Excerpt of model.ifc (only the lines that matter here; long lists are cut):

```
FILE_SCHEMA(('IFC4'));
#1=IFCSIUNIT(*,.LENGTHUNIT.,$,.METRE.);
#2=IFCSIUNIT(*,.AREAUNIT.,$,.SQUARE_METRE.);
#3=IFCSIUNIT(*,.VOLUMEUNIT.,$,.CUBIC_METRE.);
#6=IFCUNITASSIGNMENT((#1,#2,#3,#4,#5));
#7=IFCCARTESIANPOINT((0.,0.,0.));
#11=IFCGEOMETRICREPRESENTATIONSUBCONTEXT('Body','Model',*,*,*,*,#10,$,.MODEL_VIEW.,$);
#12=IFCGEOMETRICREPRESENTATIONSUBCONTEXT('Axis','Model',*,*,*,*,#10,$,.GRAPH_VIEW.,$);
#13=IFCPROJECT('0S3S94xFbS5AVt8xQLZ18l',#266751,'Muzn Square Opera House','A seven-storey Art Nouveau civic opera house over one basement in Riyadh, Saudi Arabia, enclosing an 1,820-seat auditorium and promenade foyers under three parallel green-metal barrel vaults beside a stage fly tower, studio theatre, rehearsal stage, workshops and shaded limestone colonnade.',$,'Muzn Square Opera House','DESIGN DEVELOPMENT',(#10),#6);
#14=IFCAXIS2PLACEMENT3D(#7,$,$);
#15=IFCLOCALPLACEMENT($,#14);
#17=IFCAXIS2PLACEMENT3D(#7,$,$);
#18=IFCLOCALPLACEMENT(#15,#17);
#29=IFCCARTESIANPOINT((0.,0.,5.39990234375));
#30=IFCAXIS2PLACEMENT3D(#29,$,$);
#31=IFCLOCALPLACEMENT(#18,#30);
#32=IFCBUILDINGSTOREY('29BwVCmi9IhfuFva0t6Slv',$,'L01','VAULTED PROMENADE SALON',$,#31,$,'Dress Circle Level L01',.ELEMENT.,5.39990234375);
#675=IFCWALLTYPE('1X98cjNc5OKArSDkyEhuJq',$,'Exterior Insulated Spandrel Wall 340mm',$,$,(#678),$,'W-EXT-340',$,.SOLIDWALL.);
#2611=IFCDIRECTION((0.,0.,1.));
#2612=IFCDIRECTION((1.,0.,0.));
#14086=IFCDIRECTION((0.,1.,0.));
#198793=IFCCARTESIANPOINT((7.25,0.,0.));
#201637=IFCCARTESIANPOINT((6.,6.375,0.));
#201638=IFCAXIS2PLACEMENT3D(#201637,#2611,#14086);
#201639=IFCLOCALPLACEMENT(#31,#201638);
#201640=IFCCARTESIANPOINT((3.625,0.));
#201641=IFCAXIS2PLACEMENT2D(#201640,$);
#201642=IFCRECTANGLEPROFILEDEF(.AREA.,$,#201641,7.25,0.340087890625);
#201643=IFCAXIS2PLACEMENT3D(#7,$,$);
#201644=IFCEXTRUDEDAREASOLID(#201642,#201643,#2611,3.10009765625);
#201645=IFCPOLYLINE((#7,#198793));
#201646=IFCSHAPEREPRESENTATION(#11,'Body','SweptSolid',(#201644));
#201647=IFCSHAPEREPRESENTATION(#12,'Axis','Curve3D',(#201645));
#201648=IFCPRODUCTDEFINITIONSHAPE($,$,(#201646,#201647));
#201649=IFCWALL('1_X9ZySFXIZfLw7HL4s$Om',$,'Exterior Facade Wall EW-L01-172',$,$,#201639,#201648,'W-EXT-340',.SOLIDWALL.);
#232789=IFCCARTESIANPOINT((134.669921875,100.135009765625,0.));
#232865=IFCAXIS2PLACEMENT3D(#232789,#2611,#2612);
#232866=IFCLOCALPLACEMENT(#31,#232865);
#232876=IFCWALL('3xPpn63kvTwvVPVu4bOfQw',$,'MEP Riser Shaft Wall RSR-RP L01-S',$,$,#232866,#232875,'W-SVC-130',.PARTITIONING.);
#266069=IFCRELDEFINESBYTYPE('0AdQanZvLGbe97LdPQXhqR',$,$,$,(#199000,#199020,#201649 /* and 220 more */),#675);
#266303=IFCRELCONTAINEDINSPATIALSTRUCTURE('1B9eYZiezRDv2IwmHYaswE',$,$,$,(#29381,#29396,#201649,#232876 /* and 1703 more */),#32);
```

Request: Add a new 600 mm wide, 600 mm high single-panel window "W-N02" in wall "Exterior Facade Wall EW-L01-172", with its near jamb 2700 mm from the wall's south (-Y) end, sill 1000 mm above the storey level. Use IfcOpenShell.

```python
import numpy as np
import ifcopenshell
import ifcopenshell.api.feature
import ifcopenshell.api.geometry
import ifcopenshell.api.root
import ifcopenshell.api.spatial
import ifcopenshell.geom
import ifcopenshell.util.element
import ifcopenshell.util.placement
import ifcopenshell.util.representation
import ifcopenshell.util.shape
import ifcopenshell.util.unit

model = ifcopenshell.open("model.ifc")
unit_scale = ifcopenshell.util.unit.calculate_unit_scale(model)
settings = ifcopenshell.geom.settings()


def volume(element):
    """Net volume in cubic metres, openings subtracted."""
    shape = ifcopenshell.geom.create_shape(settings, element)
    return ifcopenshell.util.shape.get_volume(shape.geometry)


wall = model.by_guid("1_X9ZySFXIZfLw7HL4s$Om")
storey = ifcopenshell.util.element.get_container(wall, ifc_class="IfcBuildingStorey")
context = ifcopenshell.util.representation.get_context(model, "Model", "Body", "MODEL_VIEW")
before = volume(wall)

width, height, from_end, sill = 0.6, 0.6, 2.7, 1  # metres

# The wall runs along its own X axis, and the end named is its -X end.
wall_shape = ifcopenshell.geom.create_shape(settings, wall)
x, y, z = ifcopenshell.util.shape.get_vertices(wall_shape.geometry).T
start = x.min() + from_end
face, thickness = float(y.min()), float(y.max() - y.min())
wall_matrix = ifcopenshell.util.placement.get_local_placement(wall.ObjectPlacement)
level = ifcopenshell.util.placement.get_local_placement(storey.ObjectPlacement)[2, 3]


def in_wall(x, y):
    """Placement at x, y metres in the wall's axes, at sill height."""
    matrix = wall_matrix.copy()
    matrix[:, 3] = wall_matrix @ np.array([x / unit_scale, y / unit_scale, 0.0, 1.0])
    matrix[2, 3] = level + sill / unit_scale
    return matrix


# Opening: a box that overshoots both wall faces by 50 mm.
opening = ifcopenshell.api.root.create_entity(model, ifc_class="IfcOpeningElement", predefined_type="OPENING")
box = ifcopenshell.api.geometry.add_wall_representation(
    model, context=context, length=width, height=height, thickness=thickness + 0.1
)
ifcopenshell.api.geometry.assign_representation(model, product=opening, representation=box)
ifcopenshell.api.geometry.edit_object_placement(model, product=opening, matrix=in_wall(start, face - 0.05), is_si=False)
ifcopenshell.api.feature.add_feature(model, feature=opening, element=wall)

window = ifcopenshell.api.root.create_entity(model, ifc_class="IfcWindow", name="W-N02", predefined_type="WINDOW")
window.OverallWidth, window.OverallHeight = width / unit_scale, height / unit_scale
window.PartitioningType = "SINGLE_PANEL"
body = ifcopenshell.api.geometry.add_window_representation(
    model,
    context=context,
    overall_width=window.OverallWidth,
    overall_height=window.OverallHeight,
    partition_type="SINGLE_PANEL",
)
ifcopenshell.api.geometry.assign_representation(model, product=window, representation=body)
ifcopenshell.api.spatial.assign_container(model, products=[window], relating_structure=storey)
ifcopenshell.api.feature.add_filling(model, opening=opening, element=window)

# Centre the window in the wall's thickness.
ifcopenshell.api.geometry.edit_object_placement(model, product=window, matrix=in_wall(start, face), is_si=False)
window_shape = ifcopenshell.geom.create_shape(settings, window)
depth = ifcopenshell.util.shape.get_vertices(window_shape.geometry)[:, 1]
offset = face + thickness / 2 - (depth.min() + depth.max()) / 2
ifcopenshell.api.geometry.edit_object_placement(model, product=window, matrix=in_wall(start, offset), is_si=False)

after = volume(wall)

print(f"wall volume {before:.3f} -> {after:.3f} m3")

model.write("model_rev.ifc")
```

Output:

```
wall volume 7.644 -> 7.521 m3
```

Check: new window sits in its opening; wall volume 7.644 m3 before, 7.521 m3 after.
